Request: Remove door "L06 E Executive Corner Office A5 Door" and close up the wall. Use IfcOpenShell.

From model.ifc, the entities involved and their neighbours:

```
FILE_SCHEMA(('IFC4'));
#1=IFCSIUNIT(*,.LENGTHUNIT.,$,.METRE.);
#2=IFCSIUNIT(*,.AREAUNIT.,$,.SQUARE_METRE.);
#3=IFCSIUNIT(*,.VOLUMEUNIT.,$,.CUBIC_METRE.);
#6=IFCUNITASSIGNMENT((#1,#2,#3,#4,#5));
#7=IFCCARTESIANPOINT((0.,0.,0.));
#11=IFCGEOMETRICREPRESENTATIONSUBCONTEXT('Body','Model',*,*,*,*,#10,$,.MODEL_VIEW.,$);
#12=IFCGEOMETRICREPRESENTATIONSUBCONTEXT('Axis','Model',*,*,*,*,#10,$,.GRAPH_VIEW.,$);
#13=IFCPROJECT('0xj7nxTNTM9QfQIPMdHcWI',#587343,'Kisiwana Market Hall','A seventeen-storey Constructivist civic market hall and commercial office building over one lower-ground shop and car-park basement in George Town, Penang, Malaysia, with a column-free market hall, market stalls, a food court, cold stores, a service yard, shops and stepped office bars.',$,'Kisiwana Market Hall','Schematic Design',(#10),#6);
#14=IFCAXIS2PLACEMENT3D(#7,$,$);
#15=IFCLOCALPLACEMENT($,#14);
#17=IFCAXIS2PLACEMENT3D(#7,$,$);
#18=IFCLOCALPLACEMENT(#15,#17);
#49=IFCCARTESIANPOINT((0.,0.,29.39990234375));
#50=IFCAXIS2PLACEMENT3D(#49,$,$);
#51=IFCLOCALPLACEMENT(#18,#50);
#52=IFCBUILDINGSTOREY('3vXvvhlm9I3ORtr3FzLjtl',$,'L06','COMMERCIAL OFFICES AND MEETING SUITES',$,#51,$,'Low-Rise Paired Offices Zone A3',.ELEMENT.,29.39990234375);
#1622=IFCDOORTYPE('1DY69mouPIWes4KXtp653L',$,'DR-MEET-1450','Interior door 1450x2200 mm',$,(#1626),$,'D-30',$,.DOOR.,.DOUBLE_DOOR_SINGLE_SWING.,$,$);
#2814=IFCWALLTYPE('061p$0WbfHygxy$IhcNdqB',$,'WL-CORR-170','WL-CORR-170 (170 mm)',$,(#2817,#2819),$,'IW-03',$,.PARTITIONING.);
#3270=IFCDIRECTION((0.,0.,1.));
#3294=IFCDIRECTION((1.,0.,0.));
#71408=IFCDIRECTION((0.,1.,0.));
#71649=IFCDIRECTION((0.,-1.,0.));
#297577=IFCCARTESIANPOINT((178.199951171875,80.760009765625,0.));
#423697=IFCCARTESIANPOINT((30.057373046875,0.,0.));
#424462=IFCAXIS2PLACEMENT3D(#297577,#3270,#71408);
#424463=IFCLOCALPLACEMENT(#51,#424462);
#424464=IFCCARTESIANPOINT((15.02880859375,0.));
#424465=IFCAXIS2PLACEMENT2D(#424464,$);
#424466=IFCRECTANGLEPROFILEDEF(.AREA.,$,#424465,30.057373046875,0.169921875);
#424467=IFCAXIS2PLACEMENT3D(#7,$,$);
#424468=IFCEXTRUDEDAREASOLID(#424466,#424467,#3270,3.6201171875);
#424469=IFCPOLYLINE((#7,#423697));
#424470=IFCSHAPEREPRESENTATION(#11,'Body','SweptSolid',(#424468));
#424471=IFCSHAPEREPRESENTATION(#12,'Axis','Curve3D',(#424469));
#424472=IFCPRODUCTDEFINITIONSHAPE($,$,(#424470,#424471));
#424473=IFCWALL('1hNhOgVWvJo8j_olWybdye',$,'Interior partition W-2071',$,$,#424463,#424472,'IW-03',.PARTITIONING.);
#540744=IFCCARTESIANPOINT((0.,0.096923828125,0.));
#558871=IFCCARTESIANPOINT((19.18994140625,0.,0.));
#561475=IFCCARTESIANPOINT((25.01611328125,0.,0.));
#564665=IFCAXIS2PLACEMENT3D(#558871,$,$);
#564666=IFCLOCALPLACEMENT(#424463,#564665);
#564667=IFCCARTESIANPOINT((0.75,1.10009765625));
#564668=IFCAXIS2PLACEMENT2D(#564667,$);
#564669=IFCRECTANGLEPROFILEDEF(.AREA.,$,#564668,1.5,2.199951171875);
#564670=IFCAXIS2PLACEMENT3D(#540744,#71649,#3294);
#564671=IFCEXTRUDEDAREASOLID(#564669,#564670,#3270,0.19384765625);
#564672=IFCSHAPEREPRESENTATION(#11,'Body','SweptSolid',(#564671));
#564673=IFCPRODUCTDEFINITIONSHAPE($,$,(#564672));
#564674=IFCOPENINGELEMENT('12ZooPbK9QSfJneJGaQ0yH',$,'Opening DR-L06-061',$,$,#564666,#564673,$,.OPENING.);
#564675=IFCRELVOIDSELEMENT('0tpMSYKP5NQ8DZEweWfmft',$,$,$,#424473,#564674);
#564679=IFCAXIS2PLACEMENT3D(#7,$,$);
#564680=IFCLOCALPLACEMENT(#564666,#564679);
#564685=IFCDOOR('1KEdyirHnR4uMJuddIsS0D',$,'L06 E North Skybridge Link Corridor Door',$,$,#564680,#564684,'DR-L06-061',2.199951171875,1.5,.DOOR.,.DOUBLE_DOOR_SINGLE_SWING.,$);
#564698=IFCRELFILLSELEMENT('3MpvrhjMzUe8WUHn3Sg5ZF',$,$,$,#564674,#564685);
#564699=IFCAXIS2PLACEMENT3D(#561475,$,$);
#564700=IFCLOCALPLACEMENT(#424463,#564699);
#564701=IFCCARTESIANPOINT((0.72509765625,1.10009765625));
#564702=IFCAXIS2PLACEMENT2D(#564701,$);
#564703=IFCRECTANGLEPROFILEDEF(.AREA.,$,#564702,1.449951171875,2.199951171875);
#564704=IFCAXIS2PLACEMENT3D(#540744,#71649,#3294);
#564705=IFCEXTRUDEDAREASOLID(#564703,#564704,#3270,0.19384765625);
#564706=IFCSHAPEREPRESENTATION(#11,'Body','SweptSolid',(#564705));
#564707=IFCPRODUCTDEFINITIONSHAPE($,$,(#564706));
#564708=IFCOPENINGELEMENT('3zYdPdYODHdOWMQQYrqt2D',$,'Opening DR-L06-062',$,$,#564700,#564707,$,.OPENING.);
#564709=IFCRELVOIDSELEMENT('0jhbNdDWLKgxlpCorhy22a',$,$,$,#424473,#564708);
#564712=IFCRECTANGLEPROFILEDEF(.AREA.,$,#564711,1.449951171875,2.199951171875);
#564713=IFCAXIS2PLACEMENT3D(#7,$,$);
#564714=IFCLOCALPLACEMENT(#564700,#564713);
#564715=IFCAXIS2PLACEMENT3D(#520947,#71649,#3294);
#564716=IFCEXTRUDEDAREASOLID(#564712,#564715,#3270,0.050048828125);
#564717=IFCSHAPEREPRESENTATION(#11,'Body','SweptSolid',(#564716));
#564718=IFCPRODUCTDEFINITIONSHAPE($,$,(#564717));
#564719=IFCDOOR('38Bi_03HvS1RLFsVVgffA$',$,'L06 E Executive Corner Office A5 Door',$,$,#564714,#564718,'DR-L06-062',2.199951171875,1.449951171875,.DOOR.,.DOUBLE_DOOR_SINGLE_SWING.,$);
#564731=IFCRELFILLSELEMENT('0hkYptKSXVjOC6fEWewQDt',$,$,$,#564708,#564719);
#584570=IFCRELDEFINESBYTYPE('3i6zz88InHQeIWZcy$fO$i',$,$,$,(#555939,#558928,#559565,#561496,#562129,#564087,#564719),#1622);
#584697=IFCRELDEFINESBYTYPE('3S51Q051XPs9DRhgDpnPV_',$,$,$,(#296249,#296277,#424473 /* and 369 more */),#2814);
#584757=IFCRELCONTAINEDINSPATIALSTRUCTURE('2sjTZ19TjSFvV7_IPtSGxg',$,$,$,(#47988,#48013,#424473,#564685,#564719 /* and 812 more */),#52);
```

```python
import ifcopenshell
import ifcopenshell.api.feature
import ifcopenshell.api.root
import ifcopenshell.geom
import ifcopenshell.util.shape

model = ifcopenshell.open("model.ifc")
settings = ifcopenshell.geom.settings()


def volume(element):
    """Net volume in cubic metres, openings subtracted."""
    shape = ifcopenshell.geom.create_shape(settings, element)
    return ifcopenshell.util.shape.get_volume(shape.geometry)


door = model.by_id(564719)
opening = door.FillsVoids[0].RelatingOpeningElement
wall = opening.VoidsElements[0].RelatingBuildingElement
before = volume(wall)

ifcopenshell.api.root.remove_product(model, product=door)
ifcopenshell.api.feature.remove_feature(model, feature=opening)

after = volume(wall)

print(f"wall volume {before:.3f} -> {after:.3f} m3")

model.write("model_v2.ifc")
```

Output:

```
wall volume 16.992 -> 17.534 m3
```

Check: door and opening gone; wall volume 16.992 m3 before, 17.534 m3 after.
